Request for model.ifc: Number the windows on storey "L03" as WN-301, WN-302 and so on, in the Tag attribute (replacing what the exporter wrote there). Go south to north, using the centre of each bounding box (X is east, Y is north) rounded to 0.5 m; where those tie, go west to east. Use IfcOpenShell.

First a look at what the model holds.

```python
import ifcopenshell
import ifcopenshell.util.element
import ifcopenshell.util.placement

model = ifcopenshell.open("model.ifc")
print(model.schema)
storey = next(s for s in model.by_type("IfcBuildingStorey") if s.Name == "L03")
windows = [e for e in ifcopenshell.util.element.get_decomposition(storey) if e.is_a("IfcWindow")]
for e in sorted(windows, key=lambda e: e.id()):
    origin = ifcopenshell.util.placement.get_local_placement(e.ObjectPlacement)[:3, 3]
    print(e.id(), e.Tag, e.Name, origin.round(2) + 0.0, sep=" | ")
```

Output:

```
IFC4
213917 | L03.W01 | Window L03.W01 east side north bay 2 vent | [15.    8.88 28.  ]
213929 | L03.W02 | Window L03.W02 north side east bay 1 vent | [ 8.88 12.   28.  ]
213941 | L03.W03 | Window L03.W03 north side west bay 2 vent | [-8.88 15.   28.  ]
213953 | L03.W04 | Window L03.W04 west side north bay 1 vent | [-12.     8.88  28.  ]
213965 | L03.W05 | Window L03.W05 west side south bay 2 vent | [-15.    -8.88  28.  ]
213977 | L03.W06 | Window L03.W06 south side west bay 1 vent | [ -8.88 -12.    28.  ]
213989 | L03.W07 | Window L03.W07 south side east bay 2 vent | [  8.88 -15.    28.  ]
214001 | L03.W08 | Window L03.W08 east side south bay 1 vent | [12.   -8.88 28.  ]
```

```python
import ifcopenshell
import ifcopenshell.geom
import ifcopenshell.util.element
import ifcopenshell.util.shape

model = ifcopenshell.open("model.ifc")
settings = ifcopenshell.geom.settings()
settings.set("use-world-coords", True)


def centre(element):
    shape = ifcopenshell.geom.create_shape(settings, element)
    return ifcopenshell.util.shape.get_bbox_centroid(shape.geometry)


storey = next(s for s in model.by_type("IfcBuildingStorey") if s.Name == "L03")
windows = [e for e in ifcopenshell.util.element.get_decomposition(storey) if e.is_a("IfcWindow")]

# Insertion points can sit at a corner or the storey origin, so sort by the geometry (in metres).
centres = {e: centre(e) for e in windows}
windows.sort(key=lambda e: (round(centres[e][1] / 0.5), centres[e][0]))

for i, e in enumerate(windows, start=1):
    number = f"WN-3{i:02d}"
    e.Tag = number
    print(e.id(), number)

model.write("model-out.ifc")
```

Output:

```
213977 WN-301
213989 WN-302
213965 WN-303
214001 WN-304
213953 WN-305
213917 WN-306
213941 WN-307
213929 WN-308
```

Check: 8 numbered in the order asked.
